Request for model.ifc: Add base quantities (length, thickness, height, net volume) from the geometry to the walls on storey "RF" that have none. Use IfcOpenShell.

First a look at what the model holds.

```python
import ifcopenshell
import ifcopenshell.util.element
import ifcopenshell.util.unit

model = ifcopenshell.open("model.ifc")
print(model.schema)
for unit_type in ("LENGTHUNIT", "AREAUNIT", "VOLUMEUNIT"):
    print(unit_type, ifcopenshell.util.unit.calculate_unit_scale(model, unit_type))
storey = next(s for s in model.by_type("IfcBuildingStorey") if s.Name == "RF")
walls = [e for e in ifcopenshell.util.element.get_decomposition(storey) if e.is_a("IfcWall")]
for e in sorted(walls, key=lambda e: e.id()):
    print(e.id(), e.is_a(), e.Name, list(ifcopenshell.util.element.get_psets(e, qtos_only=True)), sep=" | ")
```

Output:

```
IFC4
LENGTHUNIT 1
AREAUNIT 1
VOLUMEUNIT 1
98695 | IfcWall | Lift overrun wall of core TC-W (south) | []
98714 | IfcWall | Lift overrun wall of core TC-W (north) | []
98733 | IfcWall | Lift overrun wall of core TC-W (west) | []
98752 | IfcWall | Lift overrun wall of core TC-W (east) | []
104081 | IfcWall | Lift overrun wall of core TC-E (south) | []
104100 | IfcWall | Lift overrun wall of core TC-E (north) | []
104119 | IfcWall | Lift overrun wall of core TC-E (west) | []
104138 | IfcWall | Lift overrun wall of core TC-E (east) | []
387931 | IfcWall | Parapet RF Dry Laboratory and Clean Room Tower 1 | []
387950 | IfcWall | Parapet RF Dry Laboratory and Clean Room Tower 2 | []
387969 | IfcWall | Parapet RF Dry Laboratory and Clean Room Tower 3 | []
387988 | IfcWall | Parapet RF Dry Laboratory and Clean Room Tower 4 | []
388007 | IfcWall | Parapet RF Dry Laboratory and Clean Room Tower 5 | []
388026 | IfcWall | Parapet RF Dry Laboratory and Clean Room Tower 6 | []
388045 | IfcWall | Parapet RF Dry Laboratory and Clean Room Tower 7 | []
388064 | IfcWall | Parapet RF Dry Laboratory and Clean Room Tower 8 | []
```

```python
import ifcopenshell
import ifcopenshell.api.pset
import ifcopenshell.geom
import ifcopenshell.util.element
import ifcopenshell.util.shape
import ifcopenshell.util.unit

model = ifcopenshell.open("model.ifc")
unit_scale = ifcopenshell.util.unit.calculate_unit_scale(model)
volume_scale = ifcopenshell.util.unit.calculate_unit_scale(model, "VOLUMEUNIT")
settings = ifcopenshell.geom.settings()

storey = next(s for s in model.by_type("IfcBuildingStorey") if s.Name == "RF")
walls = [e for e in ifcopenshell.util.element.get_decomposition(storey) if e.is_a("IfcWall")]

for e in sorted(walls, key=lambda e: e.id()):
    if ifcopenshell.util.element.get_psets(e, qtos_only=True, should_inherit=False):
        continue
    # Geometry comes back in metres, in the element's own axes.
    shape = ifcopenshell.geom.create_shape(settings, e)
    values = {
        "Length": ifcopenshell.util.shape.get_x(shape.geometry) / unit_scale,
        "Width": ifcopenshell.util.shape.get_y(shape.geometry) / unit_scale,
        "Height": ifcopenshell.util.shape.get_z(shape.geometry) / unit_scale,
        "NetVolume": ifcopenshell.util.shape.get_volume(shape.geometry) / volume_scale,
    }
    qto = ifcopenshell.api.pset.add_qto(model, product=e, name="Qto_WallBaseQuantities")
    ifcopenshell.api.pset.edit_qto(model, qto=qto, properties=values)
    print(e.id(), {k: round(v, 3) for k, v in values.items()})

model.write("model_updated.ifc")
```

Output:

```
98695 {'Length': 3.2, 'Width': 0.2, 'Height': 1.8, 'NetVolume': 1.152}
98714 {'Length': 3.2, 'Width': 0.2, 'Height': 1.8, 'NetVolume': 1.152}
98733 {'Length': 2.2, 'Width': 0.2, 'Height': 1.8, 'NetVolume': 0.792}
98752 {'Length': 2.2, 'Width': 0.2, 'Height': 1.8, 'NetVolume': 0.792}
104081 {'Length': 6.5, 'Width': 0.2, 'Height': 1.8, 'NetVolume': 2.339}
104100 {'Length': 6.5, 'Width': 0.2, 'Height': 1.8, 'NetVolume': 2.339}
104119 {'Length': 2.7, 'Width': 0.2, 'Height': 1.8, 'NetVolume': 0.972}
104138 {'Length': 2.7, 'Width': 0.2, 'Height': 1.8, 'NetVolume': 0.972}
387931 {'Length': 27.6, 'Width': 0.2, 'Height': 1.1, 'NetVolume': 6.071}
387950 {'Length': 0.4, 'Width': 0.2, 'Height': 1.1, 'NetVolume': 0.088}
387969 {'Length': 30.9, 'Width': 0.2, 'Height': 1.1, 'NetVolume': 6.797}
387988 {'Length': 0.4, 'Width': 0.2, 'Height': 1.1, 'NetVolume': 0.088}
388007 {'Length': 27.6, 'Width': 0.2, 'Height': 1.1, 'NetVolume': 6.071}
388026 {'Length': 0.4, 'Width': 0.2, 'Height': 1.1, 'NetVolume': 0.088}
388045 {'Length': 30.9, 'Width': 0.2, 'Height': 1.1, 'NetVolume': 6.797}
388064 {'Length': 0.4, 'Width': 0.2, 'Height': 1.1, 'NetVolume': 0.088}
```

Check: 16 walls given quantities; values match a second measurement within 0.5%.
